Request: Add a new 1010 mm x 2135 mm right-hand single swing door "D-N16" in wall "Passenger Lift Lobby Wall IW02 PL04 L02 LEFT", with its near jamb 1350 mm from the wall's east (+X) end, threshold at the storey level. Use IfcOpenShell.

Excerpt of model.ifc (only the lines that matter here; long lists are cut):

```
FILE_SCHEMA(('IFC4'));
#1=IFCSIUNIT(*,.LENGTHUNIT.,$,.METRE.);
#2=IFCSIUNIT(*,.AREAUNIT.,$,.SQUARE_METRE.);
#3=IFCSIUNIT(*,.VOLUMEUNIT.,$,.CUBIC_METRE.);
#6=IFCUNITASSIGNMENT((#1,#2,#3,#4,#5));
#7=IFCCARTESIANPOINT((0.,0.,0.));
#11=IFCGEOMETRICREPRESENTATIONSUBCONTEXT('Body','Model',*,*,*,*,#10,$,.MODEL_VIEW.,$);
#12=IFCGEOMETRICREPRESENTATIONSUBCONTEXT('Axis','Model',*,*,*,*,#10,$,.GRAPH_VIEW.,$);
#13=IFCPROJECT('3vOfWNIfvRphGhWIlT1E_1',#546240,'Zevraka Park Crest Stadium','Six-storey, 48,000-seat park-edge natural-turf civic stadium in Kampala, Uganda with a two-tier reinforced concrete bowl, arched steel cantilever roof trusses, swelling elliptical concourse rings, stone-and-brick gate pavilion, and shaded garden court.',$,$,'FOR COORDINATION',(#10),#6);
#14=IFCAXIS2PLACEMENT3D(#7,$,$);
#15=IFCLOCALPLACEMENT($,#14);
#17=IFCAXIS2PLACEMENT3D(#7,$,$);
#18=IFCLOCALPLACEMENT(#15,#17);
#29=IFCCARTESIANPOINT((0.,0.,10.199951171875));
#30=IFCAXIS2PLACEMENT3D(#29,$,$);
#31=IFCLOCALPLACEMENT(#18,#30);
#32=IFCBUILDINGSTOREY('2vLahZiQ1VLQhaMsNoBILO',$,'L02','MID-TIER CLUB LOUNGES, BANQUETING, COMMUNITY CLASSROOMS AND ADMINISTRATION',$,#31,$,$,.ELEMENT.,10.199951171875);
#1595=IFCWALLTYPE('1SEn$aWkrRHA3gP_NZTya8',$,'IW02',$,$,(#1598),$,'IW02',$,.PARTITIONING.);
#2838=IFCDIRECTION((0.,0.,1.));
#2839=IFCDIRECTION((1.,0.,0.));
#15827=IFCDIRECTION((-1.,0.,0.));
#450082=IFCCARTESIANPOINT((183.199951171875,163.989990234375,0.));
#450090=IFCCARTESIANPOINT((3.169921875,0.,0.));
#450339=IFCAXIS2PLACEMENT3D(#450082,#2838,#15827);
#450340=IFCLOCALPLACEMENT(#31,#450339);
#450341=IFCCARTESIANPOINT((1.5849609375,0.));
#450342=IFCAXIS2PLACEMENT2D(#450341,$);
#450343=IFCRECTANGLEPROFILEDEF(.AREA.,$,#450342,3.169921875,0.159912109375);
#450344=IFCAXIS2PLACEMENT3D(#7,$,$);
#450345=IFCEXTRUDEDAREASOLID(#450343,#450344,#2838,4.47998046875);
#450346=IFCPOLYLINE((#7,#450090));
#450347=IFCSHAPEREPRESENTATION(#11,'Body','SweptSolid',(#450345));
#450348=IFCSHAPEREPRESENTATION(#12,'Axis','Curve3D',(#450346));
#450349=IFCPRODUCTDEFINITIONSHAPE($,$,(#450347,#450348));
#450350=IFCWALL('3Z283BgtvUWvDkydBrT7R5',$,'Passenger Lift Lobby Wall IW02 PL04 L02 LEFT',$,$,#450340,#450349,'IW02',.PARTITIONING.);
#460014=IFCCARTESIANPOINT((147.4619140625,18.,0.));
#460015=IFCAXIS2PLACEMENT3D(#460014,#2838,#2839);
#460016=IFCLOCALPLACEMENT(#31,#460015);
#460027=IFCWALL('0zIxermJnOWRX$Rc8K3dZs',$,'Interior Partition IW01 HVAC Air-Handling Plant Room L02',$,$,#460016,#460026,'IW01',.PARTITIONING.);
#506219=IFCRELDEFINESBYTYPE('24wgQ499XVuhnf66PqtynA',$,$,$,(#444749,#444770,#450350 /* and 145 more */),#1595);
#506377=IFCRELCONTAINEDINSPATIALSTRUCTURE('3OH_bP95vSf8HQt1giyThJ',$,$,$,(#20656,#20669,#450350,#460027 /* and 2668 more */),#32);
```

```python
import numpy as np
import ifcopenshell
import ifcopenshell.api.feature
import ifcopenshell.api.geometry
import ifcopenshell.api.root
import ifcopenshell.api.spatial
import ifcopenshell.geom
import ifcopenshell.util.element
import ifcopenshell.util.placement
import ifcopenshell.util.representation
import ifcopenshell.util.shape
import ifcopenshell.util.unit

model = ifcopenshell.open("model.ifc")
unit_scale = ifcopenshell.util.unit.calculate_unit_scale(model)
settings = ifcopenshell.geom.settings()


def volume(element):
    """Net volume in cubic metres, openings subtracted."""
    shape = ifcopenshell.geom.create_shape(settings, element)
    return ifcopenshell.util.shape.get_volume(shape.geometry)


wall = model.by_id(450350)
storey = ifcopenshell.util.element.get_container(wall, ifc_class="IfcBuildingStorey")
context = ifcopenshell.util.representation.get_context(model, "Model", "Body", "MODEL_VIEW")
before = volume(wall)

width, height, from_end, sill = 1.01, 2.135, 1.35, 0.0  # metres

# The wall runs along its own X axis, and the end named is its -X end.
wall_shape = ifcopenshell.geom.create_shape(settings, wall)
x, y, z = ifcopenshell.util.shape.get_vertices(wall_shape.geometry).T
start = x.min() + from_end
face, thickness = float(y.min()), float(y.max() - y.min())
wall_matrix = ifcopenshell.util.placement.get_local_placement(wall.ObjectPlacement)
level = ifcopenshell.util.placement.get_local_placement(storey.ObjectPlacement)[2, 3]


def in_wall(x, y):
    """Placement at x, y metres in the wall's axes, at sill height."""
    matrix = wall_matrix.copy()
    matrix[:, 3] = wall_matrix @ np.array([x / unit_scale, y / unit_scale, 0.0, 1.0])
    matrix[2, 3] = level + sill / unit_scale
    return matrix


# Opening: a box that overshoots both wall faces by 50 mm.
opening = ifcopenshell.api.root.create_entity(model, ifc_class="IfcOpeningElement", predefined_type="OPENING")
box = ifcopenshell.api.geometry.add_wall_representation(
    model, context=context, length=width, height=height, thickness=thickness + 0.1
)
ifcopenshell.api.geometry.assign_representation(model, product=opening, representation=box)
ifcopenshell.api.geometry.edit_object_placement(model, product=opening, matrix=in_wall(start, face - 0.05), is_si=False)
ifcopenshell.api.feature.add_feature(model, feature=opening, element=wall)

door = ifcopenshell.api.root.create_entity(model, ifc_class="IfcDoor", name="D-N16", predefined_type="DOOR")
door.OverallWidth, door.OverallHeight = width / unit_scale, height / unit_scale
door.OperationType = "SINGLE_SWING_RIGHT"
body = ifcopenshell.api.geometry.add_door_representation(
    model,
    context=context,
    overall_width=door.OverallWidth,
    overall_height=door.OverallHeight,
    operation_type="SINGLE_SWING_RIGHT",
    lining_properties={"LiningDepth": thickness / unit_scale, "ThresholdDepth": thickness / unit_scale},
)
ifcopenshell.api.geometry.assign_representation(model, product=door, representation=body)
ifcopenshell.api.spatial.assign_container(model, products=[door], relating_structure=storey)
ifcopenshell.api.feature.add_filling(model, opening=opening, element=door)

# The lining spans the wall, so the door starts at the wall face.
ifcopenshell.api.geometry.edit_object_placement(model, product=door, matrix=in_wall(start, face), is_si=False)

after = volume(wall)

print(f"wall volume {before:.3f} -> {after:.3f} m3")

model.write("model_edited.ifc")
```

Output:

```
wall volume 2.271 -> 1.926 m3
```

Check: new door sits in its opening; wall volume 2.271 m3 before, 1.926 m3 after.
